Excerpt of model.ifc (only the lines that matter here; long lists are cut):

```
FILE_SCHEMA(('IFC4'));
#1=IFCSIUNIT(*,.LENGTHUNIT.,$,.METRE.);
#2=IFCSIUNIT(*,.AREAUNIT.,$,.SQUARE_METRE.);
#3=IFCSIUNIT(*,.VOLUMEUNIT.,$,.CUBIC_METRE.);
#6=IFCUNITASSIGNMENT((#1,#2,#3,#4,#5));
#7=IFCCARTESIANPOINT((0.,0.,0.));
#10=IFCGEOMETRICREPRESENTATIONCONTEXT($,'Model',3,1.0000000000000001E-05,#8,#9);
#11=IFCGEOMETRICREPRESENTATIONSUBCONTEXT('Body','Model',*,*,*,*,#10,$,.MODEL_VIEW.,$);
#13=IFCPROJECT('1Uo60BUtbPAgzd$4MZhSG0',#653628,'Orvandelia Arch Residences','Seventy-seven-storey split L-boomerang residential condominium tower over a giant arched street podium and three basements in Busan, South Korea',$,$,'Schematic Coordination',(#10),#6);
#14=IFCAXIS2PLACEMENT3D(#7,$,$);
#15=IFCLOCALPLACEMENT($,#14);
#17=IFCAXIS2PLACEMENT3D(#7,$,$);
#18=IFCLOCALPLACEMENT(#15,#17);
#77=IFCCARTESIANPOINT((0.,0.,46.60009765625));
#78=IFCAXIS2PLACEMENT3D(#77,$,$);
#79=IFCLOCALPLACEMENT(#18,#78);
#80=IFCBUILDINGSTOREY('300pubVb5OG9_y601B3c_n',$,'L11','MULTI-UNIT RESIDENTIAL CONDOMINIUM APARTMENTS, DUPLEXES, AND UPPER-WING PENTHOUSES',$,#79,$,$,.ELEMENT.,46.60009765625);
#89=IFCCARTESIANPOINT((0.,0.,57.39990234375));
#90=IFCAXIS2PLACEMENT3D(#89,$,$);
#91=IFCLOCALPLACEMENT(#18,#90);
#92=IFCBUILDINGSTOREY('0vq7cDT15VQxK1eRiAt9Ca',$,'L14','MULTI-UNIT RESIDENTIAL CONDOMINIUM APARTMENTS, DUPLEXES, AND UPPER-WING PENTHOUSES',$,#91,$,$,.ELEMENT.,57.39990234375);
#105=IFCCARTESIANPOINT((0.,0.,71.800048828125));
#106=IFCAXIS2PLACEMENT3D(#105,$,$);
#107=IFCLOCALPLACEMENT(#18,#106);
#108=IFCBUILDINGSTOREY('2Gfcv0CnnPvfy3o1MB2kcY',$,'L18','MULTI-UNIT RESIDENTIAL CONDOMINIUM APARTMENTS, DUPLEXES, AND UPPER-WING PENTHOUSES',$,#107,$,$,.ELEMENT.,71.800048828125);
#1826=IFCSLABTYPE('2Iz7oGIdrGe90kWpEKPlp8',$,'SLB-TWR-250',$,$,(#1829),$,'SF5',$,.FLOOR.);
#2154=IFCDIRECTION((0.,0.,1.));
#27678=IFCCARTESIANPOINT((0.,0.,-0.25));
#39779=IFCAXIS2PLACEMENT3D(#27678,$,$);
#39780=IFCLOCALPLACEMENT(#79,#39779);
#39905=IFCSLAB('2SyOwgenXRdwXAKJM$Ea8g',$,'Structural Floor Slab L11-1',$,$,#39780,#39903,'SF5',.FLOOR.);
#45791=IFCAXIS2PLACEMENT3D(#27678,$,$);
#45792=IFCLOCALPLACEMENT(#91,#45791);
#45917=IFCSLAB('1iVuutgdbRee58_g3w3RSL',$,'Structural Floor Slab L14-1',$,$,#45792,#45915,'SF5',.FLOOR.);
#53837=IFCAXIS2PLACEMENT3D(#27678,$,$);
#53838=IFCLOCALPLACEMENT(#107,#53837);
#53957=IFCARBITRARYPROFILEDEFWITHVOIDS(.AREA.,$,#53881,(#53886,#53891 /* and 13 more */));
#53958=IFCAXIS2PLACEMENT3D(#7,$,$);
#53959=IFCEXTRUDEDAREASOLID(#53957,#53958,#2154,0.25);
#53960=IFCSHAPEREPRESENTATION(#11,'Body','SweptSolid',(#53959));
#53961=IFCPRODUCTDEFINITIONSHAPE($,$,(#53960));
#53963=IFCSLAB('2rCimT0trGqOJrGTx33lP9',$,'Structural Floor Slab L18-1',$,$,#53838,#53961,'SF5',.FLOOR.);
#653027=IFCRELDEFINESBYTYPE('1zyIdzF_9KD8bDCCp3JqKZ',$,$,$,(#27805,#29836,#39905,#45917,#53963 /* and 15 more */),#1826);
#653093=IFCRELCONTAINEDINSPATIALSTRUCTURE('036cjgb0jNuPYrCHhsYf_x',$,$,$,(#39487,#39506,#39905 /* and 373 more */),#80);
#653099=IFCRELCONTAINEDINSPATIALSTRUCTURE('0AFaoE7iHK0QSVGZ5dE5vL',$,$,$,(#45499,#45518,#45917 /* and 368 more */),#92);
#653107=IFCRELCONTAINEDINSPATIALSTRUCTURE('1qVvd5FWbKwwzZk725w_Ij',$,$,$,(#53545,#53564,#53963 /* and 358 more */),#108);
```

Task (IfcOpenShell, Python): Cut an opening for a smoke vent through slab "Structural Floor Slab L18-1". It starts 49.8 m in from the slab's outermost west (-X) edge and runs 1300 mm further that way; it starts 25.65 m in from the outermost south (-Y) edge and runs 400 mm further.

```python
import numpy as np
import ifcopenshell
import ifcopenshell.api.feature
import ifcopenshell.api.geometry
import ifcopenshell.api.root
import ifcopenshell.geom
import ifcopenshell.util.placement
import ifcopenshell.util.representation
import ifcopenshell.util.shape
import ifcopenshell.util.unit

model = ifcopenshell.open("model.ifc")
unit_scale = ifcopenshell.util.unit.calculate_unit_scale(model)
settings = ifcopenshell.geom.settings()


def volume(element):
    """Net volume in cubic metres, openings subtracted."""
    shape = ifcopenshell.geom.create_shape(settings, element)
    return ifcopenshell.util.shape.get_volume(shape.geometry)


slab = model.by_guid("2rCimT0trGqOJrGTx33lP9")
before = volume(slab)

# Extent in the slab's own axes, in metres. The edges named are its -X and -Y sides.
slab_shape = ifcopenshell.geom.create_shape(settings, slab)
vertices = ifcopenshell.util.shape.get_vertices(slab_shape.geometry)
x_min, y_min, bottom = vertices.min(axis=0)
top = vertices[:, 2].max()

opening = ifcopenshell.api.root.create_entity(model, ifc_class="IfcOpeningElement", name="Smoke vent opening", predefined_type="OPENING")
context = ifcopenshell.util.representation.get_context(model, "Model", "Body", "MODEL_VIEW")
width, depth = 1.3, 0.4
outline = [(0.0, 0.0), (width, 0.0), (width, depth), (0.0, depth), (0.0, 0.0)]
# Overshoot both faces by 50 mm so the cut is clean.
shape = ifcopenshell.api.geometry.add_slab_representation(
    model, context=context, depth=top - bottom + 0.1, polyline=outline
)
ifcopenshell.api.geometry.assign_representation(model, product=opening, representation=shape)

matrix = ifcopenshell.util.placement.get_local_placement(slab.ObjectPlacement)
matrix[:, 3] = matrix @ np.append(np.array([x_min + 49.8, y_min + 25.65, bottom - 0.05]) / unit_scale, 1.0)
ifcopenshell.api.geometry.edit_object_placement(model, product=opening, matrix=matrix, is_si=False)
ifcopenshell.api.feature.add_feature(model, feature=opening, element=slab)

after = volume(slab)

print(f"slab volume {before:.3f} -> {after:.3f} m3")

model.write("model_rev.ifc")
```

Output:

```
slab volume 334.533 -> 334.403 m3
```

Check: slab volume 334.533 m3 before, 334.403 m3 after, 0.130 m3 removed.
